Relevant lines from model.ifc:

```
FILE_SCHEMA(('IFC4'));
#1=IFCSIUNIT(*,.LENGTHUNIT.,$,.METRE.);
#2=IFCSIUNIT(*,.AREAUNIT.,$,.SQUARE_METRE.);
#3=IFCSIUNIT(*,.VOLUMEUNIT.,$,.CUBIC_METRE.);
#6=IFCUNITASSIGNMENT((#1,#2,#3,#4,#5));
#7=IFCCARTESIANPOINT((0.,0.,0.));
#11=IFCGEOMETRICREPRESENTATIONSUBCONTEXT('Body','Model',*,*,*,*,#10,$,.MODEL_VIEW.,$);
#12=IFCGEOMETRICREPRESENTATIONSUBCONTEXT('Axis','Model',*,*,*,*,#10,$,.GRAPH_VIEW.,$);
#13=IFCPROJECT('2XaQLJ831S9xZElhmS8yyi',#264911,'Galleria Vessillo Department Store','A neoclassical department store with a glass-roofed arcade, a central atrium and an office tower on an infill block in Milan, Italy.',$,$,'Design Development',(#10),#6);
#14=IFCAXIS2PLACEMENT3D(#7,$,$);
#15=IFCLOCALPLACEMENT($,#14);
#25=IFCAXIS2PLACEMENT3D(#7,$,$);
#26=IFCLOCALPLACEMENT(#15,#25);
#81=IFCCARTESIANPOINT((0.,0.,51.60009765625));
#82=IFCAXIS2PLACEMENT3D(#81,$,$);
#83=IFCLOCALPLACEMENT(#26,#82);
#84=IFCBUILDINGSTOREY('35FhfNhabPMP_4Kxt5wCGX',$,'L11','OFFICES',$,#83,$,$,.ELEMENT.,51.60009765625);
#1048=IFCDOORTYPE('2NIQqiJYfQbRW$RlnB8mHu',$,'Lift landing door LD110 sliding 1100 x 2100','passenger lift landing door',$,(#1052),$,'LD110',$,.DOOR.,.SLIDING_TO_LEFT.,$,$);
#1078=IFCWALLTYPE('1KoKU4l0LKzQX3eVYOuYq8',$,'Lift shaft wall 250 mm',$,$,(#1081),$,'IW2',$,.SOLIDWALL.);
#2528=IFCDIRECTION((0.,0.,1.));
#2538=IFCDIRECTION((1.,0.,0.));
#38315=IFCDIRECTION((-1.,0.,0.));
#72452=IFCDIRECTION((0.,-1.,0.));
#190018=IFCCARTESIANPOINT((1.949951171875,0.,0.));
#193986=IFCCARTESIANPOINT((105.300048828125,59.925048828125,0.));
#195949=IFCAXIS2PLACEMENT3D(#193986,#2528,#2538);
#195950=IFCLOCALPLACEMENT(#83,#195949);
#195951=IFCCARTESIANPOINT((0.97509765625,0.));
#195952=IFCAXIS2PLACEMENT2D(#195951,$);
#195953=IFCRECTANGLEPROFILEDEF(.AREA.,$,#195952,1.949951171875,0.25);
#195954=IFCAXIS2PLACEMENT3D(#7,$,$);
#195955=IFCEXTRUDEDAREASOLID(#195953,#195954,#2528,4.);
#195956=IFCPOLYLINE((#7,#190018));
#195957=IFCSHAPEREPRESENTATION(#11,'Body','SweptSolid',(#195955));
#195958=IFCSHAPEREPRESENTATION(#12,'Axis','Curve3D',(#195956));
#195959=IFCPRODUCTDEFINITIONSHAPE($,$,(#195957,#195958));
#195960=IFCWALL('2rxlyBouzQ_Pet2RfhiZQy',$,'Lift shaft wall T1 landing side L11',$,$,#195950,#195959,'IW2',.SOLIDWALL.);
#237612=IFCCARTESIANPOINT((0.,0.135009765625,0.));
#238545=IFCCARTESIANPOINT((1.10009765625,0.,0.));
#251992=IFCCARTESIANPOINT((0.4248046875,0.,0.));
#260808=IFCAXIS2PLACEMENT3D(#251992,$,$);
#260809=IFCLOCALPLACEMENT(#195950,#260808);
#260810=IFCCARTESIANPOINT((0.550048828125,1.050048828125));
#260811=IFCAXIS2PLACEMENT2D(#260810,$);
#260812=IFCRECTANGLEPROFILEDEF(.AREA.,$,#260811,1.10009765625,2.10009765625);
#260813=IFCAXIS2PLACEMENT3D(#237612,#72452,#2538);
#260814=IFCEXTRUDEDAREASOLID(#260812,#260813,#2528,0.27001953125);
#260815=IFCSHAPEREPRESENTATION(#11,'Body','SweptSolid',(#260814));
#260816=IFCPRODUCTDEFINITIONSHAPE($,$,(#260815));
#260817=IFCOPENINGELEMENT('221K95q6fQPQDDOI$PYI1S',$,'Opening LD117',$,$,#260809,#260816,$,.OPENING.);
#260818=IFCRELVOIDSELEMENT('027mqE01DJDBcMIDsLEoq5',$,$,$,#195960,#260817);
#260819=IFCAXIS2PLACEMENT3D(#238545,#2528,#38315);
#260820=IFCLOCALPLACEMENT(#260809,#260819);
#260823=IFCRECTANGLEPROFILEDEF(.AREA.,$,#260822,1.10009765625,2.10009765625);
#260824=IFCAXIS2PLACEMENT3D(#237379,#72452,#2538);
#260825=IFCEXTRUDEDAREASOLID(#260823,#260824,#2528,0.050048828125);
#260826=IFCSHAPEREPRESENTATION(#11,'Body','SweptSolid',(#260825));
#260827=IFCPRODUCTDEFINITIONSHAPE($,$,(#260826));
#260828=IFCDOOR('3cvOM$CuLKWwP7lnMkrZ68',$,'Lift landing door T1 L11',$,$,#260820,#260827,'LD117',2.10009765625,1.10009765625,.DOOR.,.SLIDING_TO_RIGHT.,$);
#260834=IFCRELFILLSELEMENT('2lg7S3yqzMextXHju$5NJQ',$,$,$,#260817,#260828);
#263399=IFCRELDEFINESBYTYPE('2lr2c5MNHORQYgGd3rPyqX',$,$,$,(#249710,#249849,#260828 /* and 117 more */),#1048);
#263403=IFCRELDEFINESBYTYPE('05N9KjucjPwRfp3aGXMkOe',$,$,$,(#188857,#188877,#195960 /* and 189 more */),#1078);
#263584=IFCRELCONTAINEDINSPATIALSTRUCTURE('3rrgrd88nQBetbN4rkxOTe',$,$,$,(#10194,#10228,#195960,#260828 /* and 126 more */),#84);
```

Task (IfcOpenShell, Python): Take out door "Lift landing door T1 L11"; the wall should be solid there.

```python
import ifcopenshell
import ifcopenshell.api.feature
import ifcopenshell.api.root
import ifcopenshell.geom
import ifcopenshell.util.shape

model = ifcopenshell.open("model.ifc")
settings = ifcopenshell.geom.settings()


def volume(element):
    """Net volume in cubic metres, openings subtracted."""
    shape = ifcopenshell.geom.create_shape(settings, element)
    return ifcopenshell.util.shape.get_volume(shape.geometry)


door = model.by_guid("3cvOM$CuLKWwP7lnMkrZ68")
opening = door.FillsVoids[0].RelatingOpeningElement
wall = opening.VoidsElements[0].RelatingBuildingElement
before = volume(wall)

ifcopenshell.api.root.remove_product(model, product=door)
ifcopenshell.api.feature.remove_feature(model, feature=opening)

after = volume(wall)

print(f"wall volume {before:.3f} -> {after:.3f} m3")

model.write("model_updated.ifc")
```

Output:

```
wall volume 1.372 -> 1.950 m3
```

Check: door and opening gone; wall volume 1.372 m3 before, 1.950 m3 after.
